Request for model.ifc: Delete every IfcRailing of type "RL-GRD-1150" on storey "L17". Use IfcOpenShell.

First a look at what the model holds.

```python
import ifcopenshell
import ifcopenshell.util.element

model = ifcopenshell.open("model.ifc")
print(model.schema)
storey = next(s for s in model.by_type("IfcBuildingStorey") if s.Name == "L17")
railings = [e for e in ifcopenshell.util.element.get_decomposition(storey) if e.is_a("IfcRailing")]
seen = {}
for e in railings:
    element_type = ifcopenshell.util.element.get_type(e)
    name = element_type.Name if element_type not in (None, e) else None
    seen[name] = seen.get(name, 0) + 1
for name, count in sorted(seen.items(), key=str):
    print(count, "x", name)
```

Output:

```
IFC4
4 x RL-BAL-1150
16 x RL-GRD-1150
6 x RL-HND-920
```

```python
import ifcopenshell
import ifcopenshell.api.root
import ifcopenshell.util.element

model = ifcopenshell.open("model.ifc")

storey = next(s for s in model.by_type("IfcBuildingStorey") if s.Name == "L17")
railings = [e for e in ifcopenshell.util.element.get_decomposition(storey) if e.is_a("IfcRailing")]
targets = [e for e in railings if (t := ifcopenshell.util.element.get_type(e)) not in (None, e) and t.Name == "RL-GRD-1150"]

for e in targets:
    ifcopenshell.api.root.remove_product(model, product=e)
print(len(targets), "removed")

model.write("model_edited.ifc")
```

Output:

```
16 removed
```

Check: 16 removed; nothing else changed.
